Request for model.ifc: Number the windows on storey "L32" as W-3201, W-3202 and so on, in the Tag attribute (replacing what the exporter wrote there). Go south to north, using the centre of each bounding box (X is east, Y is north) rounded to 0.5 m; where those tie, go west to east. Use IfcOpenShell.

First a look at what the model holds.

```python
import ifcopenshell
import ifcopenshell.util.element
import ifcopenshell.util.placement

model = ifcopenshell.open("model.ifc")
print(model.schema)
storey = next(s for s in model.by_type("IfcBuildingStorey") if s.Name == "L32")
windows = [e for e in ifcopenshell.util.element.get_decomposition(storey) if e.is_a("IfcWindow")]
for e in sorted(windows, key=lambda e: e.id()):
    origin = ifcopenshell.util.placement.get_local_placement(e.ObjectPlacement)[:3, 3]
    print(e.id(), e.Tag, e.Name, origin.round(2) + 0.0, sep=" | ")
```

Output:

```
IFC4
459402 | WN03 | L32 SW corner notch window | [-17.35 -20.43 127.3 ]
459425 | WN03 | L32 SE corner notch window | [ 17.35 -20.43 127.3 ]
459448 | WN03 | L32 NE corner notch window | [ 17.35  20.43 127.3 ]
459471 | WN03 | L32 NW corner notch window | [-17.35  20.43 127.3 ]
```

```python
import ifcopenshell
import ifcopenshell.geom
import ifcopenshell.util.element
import ifcopenshell.util.shape

model = ifcopenshell.open("model.ifc")
settings = ifcopenshell.geom.settings()
settings.set("use-world-coords", True)


def centre(element):
    shape = ifcopenshell.geom.create_shape(settings, element)
    return ifcopenshell.util.shape.get_bbox_centroid(shape.geometry)


storey = next(s for s in model.by_type("IfcBuildingStorey") if s.Name == "L32")
windows = [e for e in ifcopenshell.util.element.get_decomposition(storey) if e.is_a("IfcWindow")]

# Insertion points can sit at a corner or the storey origin, so sort by the geometry (in metres).
centres = {e: centre(e) for e in windows}
windows.sort(key=lambda e: (round(centres[e][1] / 0.5), centres[e][0]))

for i, e in enumerate(windows, start=1):
    number = f"W-32{i:02d}"
    e.Tag = number
    print(e.id(), number)

model.write("model_edited.ifc")
```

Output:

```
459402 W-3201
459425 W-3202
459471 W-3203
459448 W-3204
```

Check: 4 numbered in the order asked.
